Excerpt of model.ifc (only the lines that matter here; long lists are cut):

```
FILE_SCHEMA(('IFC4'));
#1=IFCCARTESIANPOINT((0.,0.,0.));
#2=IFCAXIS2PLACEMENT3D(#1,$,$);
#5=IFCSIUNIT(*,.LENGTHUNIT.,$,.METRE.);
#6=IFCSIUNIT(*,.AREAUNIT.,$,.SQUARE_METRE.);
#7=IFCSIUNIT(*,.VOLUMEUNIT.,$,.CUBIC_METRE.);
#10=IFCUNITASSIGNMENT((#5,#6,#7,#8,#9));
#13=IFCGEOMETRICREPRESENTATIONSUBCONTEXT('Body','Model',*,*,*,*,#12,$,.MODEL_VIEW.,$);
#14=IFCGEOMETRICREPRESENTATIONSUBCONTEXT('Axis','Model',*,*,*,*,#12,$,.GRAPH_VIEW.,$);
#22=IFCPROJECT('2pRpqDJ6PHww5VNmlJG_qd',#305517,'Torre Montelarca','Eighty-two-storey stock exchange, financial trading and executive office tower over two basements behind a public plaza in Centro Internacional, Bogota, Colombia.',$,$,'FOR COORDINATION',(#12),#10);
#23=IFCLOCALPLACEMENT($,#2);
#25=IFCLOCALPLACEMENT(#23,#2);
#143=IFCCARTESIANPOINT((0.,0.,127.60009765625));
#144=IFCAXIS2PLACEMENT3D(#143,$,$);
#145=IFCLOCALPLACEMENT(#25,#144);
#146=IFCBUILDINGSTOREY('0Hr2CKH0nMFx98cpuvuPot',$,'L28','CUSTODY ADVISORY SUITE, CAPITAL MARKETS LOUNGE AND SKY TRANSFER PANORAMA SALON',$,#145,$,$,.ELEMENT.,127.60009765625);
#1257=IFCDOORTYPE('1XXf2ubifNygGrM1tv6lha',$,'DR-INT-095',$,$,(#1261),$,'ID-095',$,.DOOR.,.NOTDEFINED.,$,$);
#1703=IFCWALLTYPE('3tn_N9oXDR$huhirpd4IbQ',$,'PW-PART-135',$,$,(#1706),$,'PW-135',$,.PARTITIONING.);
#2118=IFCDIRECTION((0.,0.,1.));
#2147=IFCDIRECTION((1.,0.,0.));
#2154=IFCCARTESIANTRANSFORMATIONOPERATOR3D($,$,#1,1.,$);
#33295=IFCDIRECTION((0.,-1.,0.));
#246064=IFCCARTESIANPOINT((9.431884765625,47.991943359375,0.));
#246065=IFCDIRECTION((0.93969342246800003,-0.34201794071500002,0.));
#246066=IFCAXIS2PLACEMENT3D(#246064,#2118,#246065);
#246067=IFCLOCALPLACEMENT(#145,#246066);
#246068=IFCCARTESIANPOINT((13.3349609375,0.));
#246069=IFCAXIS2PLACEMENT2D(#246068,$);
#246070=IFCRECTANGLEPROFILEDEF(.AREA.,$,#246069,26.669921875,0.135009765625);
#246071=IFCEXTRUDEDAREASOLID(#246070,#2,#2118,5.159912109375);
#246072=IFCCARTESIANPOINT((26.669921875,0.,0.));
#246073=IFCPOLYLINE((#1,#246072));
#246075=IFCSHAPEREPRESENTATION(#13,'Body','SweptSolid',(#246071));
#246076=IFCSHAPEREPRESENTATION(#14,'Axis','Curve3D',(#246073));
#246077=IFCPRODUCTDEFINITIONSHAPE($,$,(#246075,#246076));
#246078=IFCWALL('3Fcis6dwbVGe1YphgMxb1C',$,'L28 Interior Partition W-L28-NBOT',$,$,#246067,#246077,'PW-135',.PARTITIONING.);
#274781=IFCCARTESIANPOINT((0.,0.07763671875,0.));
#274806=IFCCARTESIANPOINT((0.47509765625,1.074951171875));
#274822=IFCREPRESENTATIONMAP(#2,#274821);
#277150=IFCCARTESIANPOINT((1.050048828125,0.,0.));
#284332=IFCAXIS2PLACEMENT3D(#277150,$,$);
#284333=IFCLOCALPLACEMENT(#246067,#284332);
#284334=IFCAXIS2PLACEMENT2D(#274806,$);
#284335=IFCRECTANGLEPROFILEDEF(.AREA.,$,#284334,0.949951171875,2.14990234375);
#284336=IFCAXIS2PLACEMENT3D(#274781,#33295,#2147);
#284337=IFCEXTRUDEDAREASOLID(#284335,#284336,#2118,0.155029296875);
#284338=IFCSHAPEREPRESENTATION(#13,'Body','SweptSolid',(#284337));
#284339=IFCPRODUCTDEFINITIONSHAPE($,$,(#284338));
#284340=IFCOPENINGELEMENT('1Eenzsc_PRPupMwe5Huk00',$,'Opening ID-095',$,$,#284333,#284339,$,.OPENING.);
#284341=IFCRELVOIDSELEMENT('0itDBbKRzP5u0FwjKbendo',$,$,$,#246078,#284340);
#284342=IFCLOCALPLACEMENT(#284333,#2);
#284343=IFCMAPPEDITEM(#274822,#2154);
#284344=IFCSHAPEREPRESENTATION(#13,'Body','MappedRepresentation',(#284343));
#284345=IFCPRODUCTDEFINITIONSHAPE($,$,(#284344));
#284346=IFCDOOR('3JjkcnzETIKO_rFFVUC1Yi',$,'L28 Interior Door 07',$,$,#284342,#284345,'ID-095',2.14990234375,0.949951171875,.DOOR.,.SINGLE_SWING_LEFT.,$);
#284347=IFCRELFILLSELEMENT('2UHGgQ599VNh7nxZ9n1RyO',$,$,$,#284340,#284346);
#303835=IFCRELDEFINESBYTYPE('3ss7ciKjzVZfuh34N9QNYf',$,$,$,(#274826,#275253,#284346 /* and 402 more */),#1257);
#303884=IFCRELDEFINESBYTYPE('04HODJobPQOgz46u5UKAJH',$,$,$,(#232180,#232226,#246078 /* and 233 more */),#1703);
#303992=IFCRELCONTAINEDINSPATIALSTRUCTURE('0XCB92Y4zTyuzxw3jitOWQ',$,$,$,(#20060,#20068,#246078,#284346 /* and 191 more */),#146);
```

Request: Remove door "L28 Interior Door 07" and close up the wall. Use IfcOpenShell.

```python
import ifcopenshell
import ifcopenshell.api.feature
import ifcopenshell.api.root
import ifcopenshell.geom
import ifcopenshell.util.shape

model = ifcopenshell.open("model.ifc")
settings = ifcopenshell.geom.settings()


def volume(element):
    """Net volume in cubic metres, openings subtracted."""
    shape = ifcopenshell.geom.create_shape(settings, element)
    return ifcopenshell.util.shape.get_volume(shape.geometry)


door = model.by_guid("3JjkcnzETIKO_rFFVUC1Yi")
opening = door.FillsVoids[0].RelatingOpeningElement
wall = opening.VoidsElements[0].RelatingBuildingElement
before = volume(wall)

ifcopenshell.api.root.remove_product(model, product=door)
ifcopenshell.api.feature.remove_feature(model, feature=opening)

after = volume(wall)

print(f"wall volume {before:.3f} -> {after:.3f} m3")

model.write("model_updated.ifc")
```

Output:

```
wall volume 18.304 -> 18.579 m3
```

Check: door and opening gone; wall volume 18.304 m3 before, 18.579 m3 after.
